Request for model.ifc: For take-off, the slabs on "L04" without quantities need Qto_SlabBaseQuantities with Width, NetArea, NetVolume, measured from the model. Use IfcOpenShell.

First a look at what the model holds.

```python
import ifcopenshell
import ifcopenshell.util.element
import ifcopenshell.util.unit

model = ifcopenshell.open("model.ifc")
print(model.schema)
for unit_type in ("LENGTHUNIT", "AREAUNIT", "VOLUMEUNIT"):
    print(unit_type, ifcopenshell.util.unit.calculate_unit_scale(model, unit_type))
storey = next(s for s in model.by_type("IfcBuildingStorey") if s.Name == "L04")
slabs = [e for e in ifcopenshell.util.element.get_decomposition(storey) if e.is_a("IfcSlab")]
for e in sorted(slabs, key=lambda e: e.id()):
    print(e.id(), e.is_a(), e.Name, list(ifcopenshell.util.element.get_psets(e, qtos_only=True)), sep=" | ")
```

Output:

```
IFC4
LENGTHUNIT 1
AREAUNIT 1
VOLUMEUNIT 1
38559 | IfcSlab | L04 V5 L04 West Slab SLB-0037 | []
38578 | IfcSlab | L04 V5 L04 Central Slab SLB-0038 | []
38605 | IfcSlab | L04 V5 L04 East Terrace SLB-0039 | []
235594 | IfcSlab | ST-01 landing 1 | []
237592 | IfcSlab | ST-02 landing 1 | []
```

```python
import ifcopenshell
import ifcopenshell.api.pset
import ifcopenshell.geom
import ifcopenshell.util.element
import ifcopenshell.util.shape
import ifcopenshell.util.unit

model = ifcopenshell.open("model.ifc")
unit_scale = ifcopenshell.util.unit.calculate_unit_scale(model)
area_scale = ifcopenshell.util.unit.calculate_unit_scale(model, "AREAUNIT")
volume_scale = ifcopenshell.util.unit.calculate_unit_scale(model, "VOLUMEUNIT")
settings = ifcopenshell.geom.settings()

storey = next(s for s in model.by_type("IfcBuildingStorey") if s.Name == "L04")
slabs = [e for e in ifcopenshell.util.element.get_decomposition(storey) if e.is_a("IfcSlab")]

for e in sorted(slabs, key=lambda e: e.id()):
    if ifcopenshell.util.element.get_psets(e, qtos_only=True, should_inherit=False):
        continue
    # Geometry comes back in metres, in the element's own axes.
    shape = ifcopenshell.geom.create_shape(settings, e)
    values = {
        "Width": ifcopenshell.util.shape.get_z(shape.geometry) / unit_scale,
        "NetArea": ifcopenshell.util.shape.get_footprint_area(shape.geometry) / area_scale,
        "NetVolume": ifcopenshell.util.shape.get_volume(shape.geometry) / volume_scale,
    }
    qto = ifcopenshell.api.pset.add_qto(model, product=e, name="Qto_SlabBaseQuantities")
    ifcopenshell.api.pset.edit_qto(model, qto=qto, properties=values)
    print(e.id(), {k: round(v, 3) for k, v in values.items()})

model.write("model_rev.ifc")
```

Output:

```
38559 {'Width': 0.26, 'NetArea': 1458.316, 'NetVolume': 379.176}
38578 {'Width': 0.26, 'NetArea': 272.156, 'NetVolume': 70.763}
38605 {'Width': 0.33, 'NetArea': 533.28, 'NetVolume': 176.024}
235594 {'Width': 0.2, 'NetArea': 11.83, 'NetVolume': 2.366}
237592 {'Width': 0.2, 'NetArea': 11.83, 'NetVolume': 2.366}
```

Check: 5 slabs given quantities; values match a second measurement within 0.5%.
